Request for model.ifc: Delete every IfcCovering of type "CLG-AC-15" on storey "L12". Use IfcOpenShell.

First a look at what the model holds.

```python
import ifcopenshell
import ifcopenshell.util.element

model = ifcopenshell.open("model.ifc")
print(model.schema)
storey = next(s for s in model.by_type("IfcBuildingStorey") if s.Name == "L12")
coverings = [e for e in ifcopenshell.util.element.get_decomposition(storey) if e.is_a("IfcCovering")]
seen = {}
for e in coverings:
    element_type = ifcopenshell.util.element.get_type(e)
    name = element_type.Name if element_type not in (None, e) else None
    seen[name] = seen.get(name, 0) + 1
for name, count in sorted(seen.items(), key=str):
    print(count, "x", name)
```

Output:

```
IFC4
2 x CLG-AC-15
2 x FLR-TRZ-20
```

```python
import ifcopenshell
import ifcopenshell.api.root
import ifcopenshell.util.element

model = ifcopenshell.open("model.ifc")

storey = next(s for s in model.by_type("IfcBuildingStorey") if s.Name == "L12")
coverings = [e for e in ifcopenshell.util.element.get_decomposition(storey) if e.is_a("IfcCovering")]
targets = [e for e in coverings if (t := ifcopenshell.util.element.get_type(e)) not in (None, e) and t.Name == "CLG-AC-15"]

for e in targets:
    ifcopenshell.api.root.remove_product(model, product=e)
print(len(targets), "removed")

model.write("model_rev.ifc")
```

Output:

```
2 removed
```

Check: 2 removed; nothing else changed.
